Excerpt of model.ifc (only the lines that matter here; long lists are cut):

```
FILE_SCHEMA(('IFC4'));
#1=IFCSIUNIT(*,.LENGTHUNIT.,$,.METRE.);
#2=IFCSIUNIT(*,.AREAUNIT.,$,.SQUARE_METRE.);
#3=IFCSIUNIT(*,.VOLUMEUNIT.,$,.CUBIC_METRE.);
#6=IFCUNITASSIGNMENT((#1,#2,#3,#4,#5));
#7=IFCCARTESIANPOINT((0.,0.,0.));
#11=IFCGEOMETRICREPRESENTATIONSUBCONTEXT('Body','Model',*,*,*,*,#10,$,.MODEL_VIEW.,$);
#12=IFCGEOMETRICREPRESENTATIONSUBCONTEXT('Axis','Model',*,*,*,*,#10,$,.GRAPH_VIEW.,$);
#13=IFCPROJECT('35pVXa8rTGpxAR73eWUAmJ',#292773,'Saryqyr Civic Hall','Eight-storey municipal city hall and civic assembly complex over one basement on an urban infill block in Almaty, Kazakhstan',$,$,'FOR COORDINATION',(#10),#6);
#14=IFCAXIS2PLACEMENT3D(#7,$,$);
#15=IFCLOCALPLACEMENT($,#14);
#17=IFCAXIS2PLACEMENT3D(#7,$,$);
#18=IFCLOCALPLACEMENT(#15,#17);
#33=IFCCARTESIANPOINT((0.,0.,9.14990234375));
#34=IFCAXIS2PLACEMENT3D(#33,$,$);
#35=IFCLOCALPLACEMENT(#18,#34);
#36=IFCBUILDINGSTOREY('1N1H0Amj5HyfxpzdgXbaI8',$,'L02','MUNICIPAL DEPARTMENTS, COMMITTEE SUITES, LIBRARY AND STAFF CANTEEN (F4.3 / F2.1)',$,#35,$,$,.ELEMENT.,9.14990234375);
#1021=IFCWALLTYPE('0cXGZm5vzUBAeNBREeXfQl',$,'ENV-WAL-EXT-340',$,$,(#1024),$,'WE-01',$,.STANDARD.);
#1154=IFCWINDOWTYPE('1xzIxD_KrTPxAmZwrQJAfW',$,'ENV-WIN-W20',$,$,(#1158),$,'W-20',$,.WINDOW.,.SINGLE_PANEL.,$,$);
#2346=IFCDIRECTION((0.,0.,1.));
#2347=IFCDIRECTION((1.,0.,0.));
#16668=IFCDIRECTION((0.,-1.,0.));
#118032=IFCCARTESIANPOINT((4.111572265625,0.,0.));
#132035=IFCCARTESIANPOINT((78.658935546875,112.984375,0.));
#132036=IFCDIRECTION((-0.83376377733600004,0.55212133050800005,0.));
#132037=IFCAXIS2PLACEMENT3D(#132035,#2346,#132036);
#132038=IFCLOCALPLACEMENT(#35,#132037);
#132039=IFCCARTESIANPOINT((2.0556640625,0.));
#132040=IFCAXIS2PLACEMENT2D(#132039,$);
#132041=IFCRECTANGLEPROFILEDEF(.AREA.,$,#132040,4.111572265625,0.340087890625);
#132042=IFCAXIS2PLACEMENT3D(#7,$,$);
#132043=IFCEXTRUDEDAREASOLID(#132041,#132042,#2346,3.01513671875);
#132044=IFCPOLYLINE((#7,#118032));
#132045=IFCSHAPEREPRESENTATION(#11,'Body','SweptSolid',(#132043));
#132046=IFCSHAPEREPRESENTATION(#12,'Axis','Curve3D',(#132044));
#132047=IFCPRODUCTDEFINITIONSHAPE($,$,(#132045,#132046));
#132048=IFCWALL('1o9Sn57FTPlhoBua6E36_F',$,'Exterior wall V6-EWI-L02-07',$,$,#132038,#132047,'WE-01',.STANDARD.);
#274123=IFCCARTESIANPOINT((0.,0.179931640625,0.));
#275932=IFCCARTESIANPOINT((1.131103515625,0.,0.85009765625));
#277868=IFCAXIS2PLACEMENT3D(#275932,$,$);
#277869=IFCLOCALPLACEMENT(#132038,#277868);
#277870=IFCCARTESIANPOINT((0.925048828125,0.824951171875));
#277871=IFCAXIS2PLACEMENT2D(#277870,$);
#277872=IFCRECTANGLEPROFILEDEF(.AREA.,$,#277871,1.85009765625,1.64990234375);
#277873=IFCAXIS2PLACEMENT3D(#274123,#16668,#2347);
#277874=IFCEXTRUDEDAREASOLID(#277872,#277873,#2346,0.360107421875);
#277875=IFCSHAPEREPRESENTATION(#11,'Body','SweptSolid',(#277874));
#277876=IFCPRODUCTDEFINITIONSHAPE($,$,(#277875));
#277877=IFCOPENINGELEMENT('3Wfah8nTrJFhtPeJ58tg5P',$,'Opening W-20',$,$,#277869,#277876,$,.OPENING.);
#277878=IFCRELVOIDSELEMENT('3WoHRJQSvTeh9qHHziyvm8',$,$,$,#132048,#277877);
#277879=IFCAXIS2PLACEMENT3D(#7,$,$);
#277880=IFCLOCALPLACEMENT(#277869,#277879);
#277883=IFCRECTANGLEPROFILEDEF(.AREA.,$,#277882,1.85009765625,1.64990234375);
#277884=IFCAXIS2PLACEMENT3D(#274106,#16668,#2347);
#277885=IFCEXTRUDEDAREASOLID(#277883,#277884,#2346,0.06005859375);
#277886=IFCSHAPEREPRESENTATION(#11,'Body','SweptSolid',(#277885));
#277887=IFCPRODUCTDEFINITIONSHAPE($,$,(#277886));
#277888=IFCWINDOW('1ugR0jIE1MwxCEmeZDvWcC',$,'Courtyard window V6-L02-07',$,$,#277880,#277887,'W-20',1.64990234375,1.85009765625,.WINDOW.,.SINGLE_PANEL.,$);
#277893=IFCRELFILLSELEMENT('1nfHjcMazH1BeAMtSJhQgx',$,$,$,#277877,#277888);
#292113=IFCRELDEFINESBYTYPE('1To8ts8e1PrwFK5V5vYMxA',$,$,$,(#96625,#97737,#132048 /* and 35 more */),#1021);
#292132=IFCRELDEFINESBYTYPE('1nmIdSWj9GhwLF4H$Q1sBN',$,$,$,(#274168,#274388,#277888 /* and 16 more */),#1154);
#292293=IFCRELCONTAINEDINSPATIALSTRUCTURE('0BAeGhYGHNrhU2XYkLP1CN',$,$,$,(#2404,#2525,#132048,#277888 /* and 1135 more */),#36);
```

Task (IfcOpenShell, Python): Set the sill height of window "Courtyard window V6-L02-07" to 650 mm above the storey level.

```python
import numpy as np
import ifcopenshell
import ifcopenshell.api.geometry
import ifcopenshell.geom
import ifcopenshell.util.element
import ifcopenshell.util.placement
import ifcopenshell.util.shape
import ifcopenshell.util.unit

model = ifcopenshell.open("model.ifc")
unit_scale = ifcopenshell.util.unit.calculate_unit_scale(model)

window = model.by_guid("1ugR0jIE1MwxCEmeZDvWcC")
opening = window.FillsVoids[0].RelatingOpeningElement
storey = ifcopenshell.util.element.get_container(window, ifc_class="IfcBuildingStorey")
level = ifcopenshell.util.placement.get_local_placement(storey.ObjectPlacement)[2, 3]

# The opening's origin need not be at the sill, so measure its lowest point.
shape = ifcopenshell.geom.create_shape(ifcopenshell.geom.settings(), opening)
bottom = ifcopenshell.util.shape.get_shape_bottom_elevation(shape, shape.geometry) / unit_scale
dz = level + 0.65 - bottom

shift = np.array([0.0, 0.0, dz])
# The window is placed relative to its opening, so it follows when the opening moves.
matrix = ifcopenshell.util.placement.get_local_placement(opening.ObjectPlacement)
matrix[:3, 3] += shift
ifcopenshell.api.geometry.edit_object_placement(
    model, product=opening, matrix=matrix, is_si=False, should_transform_children=True
)

print(f"moved by {dz * unit_scale:+.3f} m")

model.write("model_rev.ifc")
```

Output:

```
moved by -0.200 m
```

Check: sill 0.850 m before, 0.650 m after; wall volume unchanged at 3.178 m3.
